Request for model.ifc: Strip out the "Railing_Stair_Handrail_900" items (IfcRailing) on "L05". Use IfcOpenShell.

First a look at what the model holds.

```python
import ifcopenshell
import ifcopenshell.util.element

model = ifcopenshell.open("model.ifc")
print(model.schema)
storey = next(s for s in model.by_type("IfcBuildingStorey") if s.Name == "L05")
railings = [e for e in ifcopenshell.util.element.get_decomposition(storey) if e.is_a("IfcRailing")]
seen = {}
for e in railings:
    element_type = ifcopenshell.util.element.get_type(e)
    name = element_type.Name if element_type not in (None, e) else None
    seen[name] = seen.get(name, 0) + 1
for name, count in sorted(seen.items(), key=str):
    print(count, "x", name)
```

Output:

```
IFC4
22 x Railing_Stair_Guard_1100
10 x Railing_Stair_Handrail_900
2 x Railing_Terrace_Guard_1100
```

```python
import ifcopenshell
import ifcopenshell.api.root
import ifcopenshell.util.element

model = ifcopenshell.open("model.ifc")

storey = next(s for s in model.by_type("IfcBuildingStorey") if s.Name == "L05")
railings = [e for e in ifcopenshell.util.element.get_decomposition(storey) if e.is_a("IfcRailing")]
targets = [e for e in railings if (t := ifcopenshell.util.element.get_type(e)) not in (None, e) and t.Name == "Railing_Stair_Handrail_900"]

for e in targets:
    ifcopenshell.api.root.remove_product(model, product=e)
print(len(targets), "removed")

model.write("model_updated.ifc")
```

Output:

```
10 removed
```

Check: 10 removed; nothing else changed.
